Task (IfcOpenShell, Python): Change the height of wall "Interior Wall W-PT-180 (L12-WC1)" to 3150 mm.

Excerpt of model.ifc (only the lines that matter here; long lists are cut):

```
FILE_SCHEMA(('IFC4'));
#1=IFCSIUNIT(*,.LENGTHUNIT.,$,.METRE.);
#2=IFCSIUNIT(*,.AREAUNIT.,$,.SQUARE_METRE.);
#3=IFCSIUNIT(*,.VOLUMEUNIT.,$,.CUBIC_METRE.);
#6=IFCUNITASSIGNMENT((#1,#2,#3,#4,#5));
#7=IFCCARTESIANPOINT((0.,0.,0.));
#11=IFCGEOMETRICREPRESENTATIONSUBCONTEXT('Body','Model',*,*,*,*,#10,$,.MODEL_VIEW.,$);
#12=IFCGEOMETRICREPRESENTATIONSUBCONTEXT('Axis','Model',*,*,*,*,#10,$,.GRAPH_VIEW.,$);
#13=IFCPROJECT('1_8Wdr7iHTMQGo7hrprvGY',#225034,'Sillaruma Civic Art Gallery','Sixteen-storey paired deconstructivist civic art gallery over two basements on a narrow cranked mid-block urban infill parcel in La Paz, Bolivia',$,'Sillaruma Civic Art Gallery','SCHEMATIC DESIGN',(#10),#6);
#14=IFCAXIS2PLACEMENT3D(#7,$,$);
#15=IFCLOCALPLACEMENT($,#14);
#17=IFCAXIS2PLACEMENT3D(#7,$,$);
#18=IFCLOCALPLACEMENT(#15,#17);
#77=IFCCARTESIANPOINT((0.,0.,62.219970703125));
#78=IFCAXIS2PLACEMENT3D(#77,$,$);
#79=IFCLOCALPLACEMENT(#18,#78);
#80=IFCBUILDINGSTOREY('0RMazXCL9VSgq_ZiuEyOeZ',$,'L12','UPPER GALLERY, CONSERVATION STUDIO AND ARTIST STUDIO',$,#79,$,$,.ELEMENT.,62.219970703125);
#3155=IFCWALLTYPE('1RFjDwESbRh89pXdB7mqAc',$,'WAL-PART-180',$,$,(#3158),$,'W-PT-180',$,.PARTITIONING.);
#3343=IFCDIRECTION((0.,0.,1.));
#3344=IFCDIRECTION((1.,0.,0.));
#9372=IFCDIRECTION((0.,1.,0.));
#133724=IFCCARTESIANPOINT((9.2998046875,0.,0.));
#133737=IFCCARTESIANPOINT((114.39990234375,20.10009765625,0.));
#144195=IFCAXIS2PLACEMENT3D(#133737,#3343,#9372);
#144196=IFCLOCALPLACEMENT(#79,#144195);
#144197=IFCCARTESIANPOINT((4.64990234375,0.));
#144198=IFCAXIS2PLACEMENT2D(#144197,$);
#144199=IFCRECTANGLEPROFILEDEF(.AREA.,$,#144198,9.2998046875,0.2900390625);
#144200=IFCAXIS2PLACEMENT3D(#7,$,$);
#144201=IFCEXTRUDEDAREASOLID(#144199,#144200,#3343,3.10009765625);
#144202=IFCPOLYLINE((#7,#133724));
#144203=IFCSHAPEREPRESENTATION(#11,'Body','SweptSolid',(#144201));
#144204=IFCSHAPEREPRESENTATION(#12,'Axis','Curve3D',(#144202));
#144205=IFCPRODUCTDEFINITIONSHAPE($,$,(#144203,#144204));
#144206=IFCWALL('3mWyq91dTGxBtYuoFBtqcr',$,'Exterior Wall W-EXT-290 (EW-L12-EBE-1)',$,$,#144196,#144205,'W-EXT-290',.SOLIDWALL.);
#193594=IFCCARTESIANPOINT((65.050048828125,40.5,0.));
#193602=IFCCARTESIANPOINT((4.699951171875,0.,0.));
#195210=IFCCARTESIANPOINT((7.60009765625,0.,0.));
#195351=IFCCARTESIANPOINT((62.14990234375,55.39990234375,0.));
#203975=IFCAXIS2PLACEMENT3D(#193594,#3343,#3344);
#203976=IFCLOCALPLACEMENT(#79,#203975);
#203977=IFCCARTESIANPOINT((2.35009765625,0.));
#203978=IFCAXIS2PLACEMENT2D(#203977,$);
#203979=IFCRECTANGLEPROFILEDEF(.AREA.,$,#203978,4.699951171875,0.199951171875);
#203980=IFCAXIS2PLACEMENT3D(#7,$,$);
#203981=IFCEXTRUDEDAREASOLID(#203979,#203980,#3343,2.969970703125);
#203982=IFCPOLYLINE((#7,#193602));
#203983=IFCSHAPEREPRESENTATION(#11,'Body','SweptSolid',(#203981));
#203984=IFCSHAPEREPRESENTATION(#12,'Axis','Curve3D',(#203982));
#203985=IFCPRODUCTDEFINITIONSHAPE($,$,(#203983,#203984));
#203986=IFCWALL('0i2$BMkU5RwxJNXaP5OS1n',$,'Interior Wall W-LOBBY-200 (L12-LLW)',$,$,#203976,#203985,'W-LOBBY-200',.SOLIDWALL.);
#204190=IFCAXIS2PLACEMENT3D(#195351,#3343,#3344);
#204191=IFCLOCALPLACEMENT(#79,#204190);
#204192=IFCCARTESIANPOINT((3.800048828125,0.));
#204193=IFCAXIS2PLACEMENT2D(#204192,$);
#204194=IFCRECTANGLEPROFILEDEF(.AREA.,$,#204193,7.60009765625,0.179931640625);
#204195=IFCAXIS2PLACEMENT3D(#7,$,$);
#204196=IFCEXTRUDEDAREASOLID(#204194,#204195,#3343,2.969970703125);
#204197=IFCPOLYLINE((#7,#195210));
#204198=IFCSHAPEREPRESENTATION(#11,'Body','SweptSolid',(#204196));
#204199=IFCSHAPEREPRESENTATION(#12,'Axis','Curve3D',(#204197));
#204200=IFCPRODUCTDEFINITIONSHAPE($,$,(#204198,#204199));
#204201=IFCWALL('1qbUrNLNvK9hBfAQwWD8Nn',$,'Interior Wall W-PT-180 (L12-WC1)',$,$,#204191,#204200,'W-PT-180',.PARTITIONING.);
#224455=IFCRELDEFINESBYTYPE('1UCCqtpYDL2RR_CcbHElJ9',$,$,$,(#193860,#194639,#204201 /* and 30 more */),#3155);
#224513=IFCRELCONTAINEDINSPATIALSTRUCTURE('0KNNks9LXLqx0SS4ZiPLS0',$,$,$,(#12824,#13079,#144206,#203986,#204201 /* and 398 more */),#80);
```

```python
import ifcopenshell
import ifcopenshell.geom
import ifcopenshell.util.representation
import ifcopenshell.util.shape
import ifcopenshell.util.unit

model = ifcopenshell.open("model.ifc")
unit_scale = ifcopenshell.util.unit.calculate_unit_scale(model)
settings = ifcopenshell.geom.settings()


def volume(element):
    """Net volume in cubic metres, openings subtracted."""
    shape = ifcopenshell.geom.create_shape(settings, element)
    return ifcopenshell.util.shape.get_volume(shape.geometry)


wall = model.by_id(204201)
before = volume(wall)

body = ifcopenshell.util.representation.get_representation(wall, "Model", "Body")
solid = body.Items[0]
old_height = solid.Depth
solid.Depth = 3.15 / unit_scale
after = volume(wall)

print(f"height {old_height:g} -> {solid.Depth:g}, volume {before:.3f} -> {after:.3f} m3")

model.write("model_edited.ifc")
```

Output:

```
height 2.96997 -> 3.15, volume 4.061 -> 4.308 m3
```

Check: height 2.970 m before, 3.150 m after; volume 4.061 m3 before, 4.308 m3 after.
